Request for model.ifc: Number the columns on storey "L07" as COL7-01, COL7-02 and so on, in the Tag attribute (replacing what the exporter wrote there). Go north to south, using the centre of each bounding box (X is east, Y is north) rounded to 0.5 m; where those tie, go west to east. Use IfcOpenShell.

First a look at what the model holds.

```python
import ifcopenshell
import ifcopenshell.util.element
import ifcopenshell.util.placement

model = ifcopenshell.open("model.ifc")
print(model.schema)
storey = next(s for s in model.by_type("IfcBuildingStorey") if s.Name == "L07")
columns = [e for e in ifcopenshell.util.element.get_decomposition(storey) if e.is_a("IfcColumn")]
for e in sorted(columns, key=lambda e: e.id()):
    origin = ifcopenshell.util.placement.get_local_placement(e.ObjectPlacement)[:3, 3]
    print(e.id(), e.Tag, e.Name, origin.round(2) + 0.0, sep=" | ")
```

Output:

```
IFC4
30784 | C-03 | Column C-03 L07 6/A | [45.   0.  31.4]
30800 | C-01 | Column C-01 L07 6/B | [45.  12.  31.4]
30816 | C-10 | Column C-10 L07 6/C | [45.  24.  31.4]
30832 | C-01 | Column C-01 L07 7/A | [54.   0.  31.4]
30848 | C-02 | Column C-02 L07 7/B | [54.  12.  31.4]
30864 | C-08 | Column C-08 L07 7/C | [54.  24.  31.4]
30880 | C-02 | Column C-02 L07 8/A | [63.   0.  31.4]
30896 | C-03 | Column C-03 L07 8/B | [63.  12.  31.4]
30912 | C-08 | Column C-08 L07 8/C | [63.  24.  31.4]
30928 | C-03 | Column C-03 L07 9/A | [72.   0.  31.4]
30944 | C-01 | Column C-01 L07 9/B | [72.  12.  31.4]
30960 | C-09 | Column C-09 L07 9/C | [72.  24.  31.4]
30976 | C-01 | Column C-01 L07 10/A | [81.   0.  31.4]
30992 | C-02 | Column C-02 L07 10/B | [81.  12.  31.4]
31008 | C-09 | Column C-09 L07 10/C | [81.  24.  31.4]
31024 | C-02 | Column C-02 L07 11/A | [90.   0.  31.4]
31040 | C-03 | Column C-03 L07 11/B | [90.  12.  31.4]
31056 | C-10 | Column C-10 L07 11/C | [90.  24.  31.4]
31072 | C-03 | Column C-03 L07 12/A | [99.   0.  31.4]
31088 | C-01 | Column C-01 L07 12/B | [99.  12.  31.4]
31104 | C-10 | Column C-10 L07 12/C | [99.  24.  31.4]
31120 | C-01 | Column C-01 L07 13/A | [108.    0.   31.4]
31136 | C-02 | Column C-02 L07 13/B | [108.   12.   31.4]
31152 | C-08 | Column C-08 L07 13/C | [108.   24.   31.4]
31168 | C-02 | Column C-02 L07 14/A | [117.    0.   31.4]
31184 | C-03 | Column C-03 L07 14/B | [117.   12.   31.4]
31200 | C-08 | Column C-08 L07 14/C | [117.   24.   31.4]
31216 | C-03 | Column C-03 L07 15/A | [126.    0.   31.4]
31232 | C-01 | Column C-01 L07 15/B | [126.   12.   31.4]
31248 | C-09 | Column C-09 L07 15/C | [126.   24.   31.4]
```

```python
import ifcopenshell
import ifcopenshell.geom
import ifcopenshell.util.element
import ifcopenshell.util.shape

model = ifcopenshell.open("model.ifc")
settings = ifcopenshell.geom.settings()
settings.set("use-world-coords", True)


def centre(element):
    shape = ifcopenshell.geom.create_shape(settings, element)
    return ifcopenshell.util.shape.get_bbox_centroid(shape.geometry)


storey = next(s for s in model.by_type("IfcBuildingStorey") if s.Name == "L07")
columns = [e for e in ifcopenshell.util.element.get_decomposition(storey) if e.is_a("IfcColumn")]

# Insertion points can sit at a corner or the storey origin, so sort by the geometry (in metres).
centres = {e: centre(e) for e in columns}
columns.sort(key=lambda e: (-round(centres[e][1] / 0.5), centres[e][0]))

for i, e in enumerate(columns, start=1):
    number = f"COL7-{i:02d}"
    e.Tag = number
    print(e.id(), number)

model.write("model_v2.ifc")
```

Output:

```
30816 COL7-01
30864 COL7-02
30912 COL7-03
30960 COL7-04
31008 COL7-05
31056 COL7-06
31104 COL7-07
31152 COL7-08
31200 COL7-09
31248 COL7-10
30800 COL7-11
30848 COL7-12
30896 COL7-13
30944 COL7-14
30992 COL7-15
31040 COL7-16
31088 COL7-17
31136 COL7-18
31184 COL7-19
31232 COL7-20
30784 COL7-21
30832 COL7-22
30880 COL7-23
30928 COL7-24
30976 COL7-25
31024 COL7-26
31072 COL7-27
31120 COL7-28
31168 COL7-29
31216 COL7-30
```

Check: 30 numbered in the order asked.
